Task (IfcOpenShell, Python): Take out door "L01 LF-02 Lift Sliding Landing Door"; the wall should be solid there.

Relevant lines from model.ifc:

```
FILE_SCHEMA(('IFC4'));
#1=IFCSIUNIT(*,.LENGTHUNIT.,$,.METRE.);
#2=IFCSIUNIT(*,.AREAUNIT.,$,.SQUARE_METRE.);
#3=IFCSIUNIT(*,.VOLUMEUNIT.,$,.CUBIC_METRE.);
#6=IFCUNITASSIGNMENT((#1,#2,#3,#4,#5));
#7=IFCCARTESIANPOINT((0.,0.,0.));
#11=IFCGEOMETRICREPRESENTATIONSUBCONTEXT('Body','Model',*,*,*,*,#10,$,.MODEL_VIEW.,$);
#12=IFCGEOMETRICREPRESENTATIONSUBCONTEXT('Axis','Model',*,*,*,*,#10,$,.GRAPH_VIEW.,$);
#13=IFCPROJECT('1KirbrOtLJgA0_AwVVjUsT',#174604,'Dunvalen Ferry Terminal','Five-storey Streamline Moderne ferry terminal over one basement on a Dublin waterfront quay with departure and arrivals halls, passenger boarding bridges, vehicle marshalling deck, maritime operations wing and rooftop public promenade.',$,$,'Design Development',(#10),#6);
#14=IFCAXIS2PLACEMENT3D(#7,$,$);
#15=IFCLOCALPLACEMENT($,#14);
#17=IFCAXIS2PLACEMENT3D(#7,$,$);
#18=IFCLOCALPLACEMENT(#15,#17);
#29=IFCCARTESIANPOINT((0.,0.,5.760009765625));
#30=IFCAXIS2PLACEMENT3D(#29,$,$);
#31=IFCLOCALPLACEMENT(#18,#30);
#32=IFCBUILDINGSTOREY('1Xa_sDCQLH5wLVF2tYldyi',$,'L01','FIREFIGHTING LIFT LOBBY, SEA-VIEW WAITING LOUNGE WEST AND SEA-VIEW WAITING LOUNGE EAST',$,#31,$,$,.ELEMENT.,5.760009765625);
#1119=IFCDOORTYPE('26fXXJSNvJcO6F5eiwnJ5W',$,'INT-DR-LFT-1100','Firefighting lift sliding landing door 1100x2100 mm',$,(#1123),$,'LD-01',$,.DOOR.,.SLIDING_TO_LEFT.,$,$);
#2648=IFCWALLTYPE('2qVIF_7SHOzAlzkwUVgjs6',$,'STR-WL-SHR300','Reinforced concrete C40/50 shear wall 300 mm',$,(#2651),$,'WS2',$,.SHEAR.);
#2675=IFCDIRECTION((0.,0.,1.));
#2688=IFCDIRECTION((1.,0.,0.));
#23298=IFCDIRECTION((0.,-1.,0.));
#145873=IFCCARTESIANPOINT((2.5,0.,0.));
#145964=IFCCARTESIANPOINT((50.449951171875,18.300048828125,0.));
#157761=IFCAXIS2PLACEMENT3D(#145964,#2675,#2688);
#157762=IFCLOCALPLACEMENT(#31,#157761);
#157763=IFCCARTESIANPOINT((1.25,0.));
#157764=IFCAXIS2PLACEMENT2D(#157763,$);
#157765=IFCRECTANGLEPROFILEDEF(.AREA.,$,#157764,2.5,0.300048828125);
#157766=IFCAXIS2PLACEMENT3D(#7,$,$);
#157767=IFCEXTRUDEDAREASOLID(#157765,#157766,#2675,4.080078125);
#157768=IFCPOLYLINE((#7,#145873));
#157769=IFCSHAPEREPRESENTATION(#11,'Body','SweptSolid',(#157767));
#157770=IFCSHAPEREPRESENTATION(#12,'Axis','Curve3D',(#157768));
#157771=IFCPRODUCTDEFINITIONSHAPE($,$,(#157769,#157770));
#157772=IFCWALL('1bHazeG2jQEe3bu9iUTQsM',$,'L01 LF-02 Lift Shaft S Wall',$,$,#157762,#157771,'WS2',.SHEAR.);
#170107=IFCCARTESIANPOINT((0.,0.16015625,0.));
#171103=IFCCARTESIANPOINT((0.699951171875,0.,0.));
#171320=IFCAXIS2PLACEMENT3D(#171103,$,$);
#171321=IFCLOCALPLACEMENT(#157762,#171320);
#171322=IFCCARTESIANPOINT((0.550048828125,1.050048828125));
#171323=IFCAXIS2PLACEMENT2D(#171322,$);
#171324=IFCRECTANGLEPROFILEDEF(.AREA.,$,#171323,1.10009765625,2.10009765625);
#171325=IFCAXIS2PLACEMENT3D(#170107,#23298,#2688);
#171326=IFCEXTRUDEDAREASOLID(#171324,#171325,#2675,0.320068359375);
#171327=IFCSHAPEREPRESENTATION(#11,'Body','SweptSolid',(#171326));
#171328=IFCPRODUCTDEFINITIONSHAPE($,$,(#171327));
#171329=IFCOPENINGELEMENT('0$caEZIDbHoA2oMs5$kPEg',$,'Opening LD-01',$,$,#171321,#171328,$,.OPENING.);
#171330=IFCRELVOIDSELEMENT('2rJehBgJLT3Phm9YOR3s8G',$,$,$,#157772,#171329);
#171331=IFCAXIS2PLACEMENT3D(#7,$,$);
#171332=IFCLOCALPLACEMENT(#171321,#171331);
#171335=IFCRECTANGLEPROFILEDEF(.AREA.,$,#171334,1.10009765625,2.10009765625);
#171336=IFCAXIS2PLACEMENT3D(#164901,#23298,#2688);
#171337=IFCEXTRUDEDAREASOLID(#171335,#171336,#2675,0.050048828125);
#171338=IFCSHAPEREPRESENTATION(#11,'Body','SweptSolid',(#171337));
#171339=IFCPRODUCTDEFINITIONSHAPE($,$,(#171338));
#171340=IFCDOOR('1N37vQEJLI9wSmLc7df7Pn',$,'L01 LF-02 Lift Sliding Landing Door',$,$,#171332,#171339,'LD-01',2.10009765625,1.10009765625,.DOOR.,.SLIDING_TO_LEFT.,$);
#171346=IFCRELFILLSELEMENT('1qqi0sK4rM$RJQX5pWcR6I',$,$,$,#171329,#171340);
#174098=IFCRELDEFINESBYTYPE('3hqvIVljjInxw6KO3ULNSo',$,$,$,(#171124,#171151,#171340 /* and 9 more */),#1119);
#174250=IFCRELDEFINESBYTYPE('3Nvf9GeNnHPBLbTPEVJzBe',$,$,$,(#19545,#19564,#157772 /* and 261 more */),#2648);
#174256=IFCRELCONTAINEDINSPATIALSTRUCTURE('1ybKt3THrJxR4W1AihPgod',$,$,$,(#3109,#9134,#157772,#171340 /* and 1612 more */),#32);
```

```python
import ifcopenshell
import ifcopenshell.api.feature
import ifcopenshell.api.root
import ifcopenshell.geom
import ifcopenshell.util.shape

model = ifcopenshell.open("model.ifc")
settings = ifcopenshell.geom.settings()


def volume(element):
    """Net volume in cubic metres, openings subtracted."""
    shape = ifcopenshell.geom.create_shape(settings, element)
    return ifcopenshell.util.shape.get_volume(shape.geometry)


door = model.by_id(171340)
opening = door.FillsVoids[0].RelatingOpeningElement
wall = opening.VoidsElements[0].RelatingBuildingElement
before = volume(wall)

ifcopenshell.api.root.remove_product(model, product=door)
ifcopenshell.api.feature.remove_feature(model, feature=opening)

after = volume(wall)

print(f"wall volume {before:.3f} -> {after:.3f} m3")

model.write("model_updated.ifc")
```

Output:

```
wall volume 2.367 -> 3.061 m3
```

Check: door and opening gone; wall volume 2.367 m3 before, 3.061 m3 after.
